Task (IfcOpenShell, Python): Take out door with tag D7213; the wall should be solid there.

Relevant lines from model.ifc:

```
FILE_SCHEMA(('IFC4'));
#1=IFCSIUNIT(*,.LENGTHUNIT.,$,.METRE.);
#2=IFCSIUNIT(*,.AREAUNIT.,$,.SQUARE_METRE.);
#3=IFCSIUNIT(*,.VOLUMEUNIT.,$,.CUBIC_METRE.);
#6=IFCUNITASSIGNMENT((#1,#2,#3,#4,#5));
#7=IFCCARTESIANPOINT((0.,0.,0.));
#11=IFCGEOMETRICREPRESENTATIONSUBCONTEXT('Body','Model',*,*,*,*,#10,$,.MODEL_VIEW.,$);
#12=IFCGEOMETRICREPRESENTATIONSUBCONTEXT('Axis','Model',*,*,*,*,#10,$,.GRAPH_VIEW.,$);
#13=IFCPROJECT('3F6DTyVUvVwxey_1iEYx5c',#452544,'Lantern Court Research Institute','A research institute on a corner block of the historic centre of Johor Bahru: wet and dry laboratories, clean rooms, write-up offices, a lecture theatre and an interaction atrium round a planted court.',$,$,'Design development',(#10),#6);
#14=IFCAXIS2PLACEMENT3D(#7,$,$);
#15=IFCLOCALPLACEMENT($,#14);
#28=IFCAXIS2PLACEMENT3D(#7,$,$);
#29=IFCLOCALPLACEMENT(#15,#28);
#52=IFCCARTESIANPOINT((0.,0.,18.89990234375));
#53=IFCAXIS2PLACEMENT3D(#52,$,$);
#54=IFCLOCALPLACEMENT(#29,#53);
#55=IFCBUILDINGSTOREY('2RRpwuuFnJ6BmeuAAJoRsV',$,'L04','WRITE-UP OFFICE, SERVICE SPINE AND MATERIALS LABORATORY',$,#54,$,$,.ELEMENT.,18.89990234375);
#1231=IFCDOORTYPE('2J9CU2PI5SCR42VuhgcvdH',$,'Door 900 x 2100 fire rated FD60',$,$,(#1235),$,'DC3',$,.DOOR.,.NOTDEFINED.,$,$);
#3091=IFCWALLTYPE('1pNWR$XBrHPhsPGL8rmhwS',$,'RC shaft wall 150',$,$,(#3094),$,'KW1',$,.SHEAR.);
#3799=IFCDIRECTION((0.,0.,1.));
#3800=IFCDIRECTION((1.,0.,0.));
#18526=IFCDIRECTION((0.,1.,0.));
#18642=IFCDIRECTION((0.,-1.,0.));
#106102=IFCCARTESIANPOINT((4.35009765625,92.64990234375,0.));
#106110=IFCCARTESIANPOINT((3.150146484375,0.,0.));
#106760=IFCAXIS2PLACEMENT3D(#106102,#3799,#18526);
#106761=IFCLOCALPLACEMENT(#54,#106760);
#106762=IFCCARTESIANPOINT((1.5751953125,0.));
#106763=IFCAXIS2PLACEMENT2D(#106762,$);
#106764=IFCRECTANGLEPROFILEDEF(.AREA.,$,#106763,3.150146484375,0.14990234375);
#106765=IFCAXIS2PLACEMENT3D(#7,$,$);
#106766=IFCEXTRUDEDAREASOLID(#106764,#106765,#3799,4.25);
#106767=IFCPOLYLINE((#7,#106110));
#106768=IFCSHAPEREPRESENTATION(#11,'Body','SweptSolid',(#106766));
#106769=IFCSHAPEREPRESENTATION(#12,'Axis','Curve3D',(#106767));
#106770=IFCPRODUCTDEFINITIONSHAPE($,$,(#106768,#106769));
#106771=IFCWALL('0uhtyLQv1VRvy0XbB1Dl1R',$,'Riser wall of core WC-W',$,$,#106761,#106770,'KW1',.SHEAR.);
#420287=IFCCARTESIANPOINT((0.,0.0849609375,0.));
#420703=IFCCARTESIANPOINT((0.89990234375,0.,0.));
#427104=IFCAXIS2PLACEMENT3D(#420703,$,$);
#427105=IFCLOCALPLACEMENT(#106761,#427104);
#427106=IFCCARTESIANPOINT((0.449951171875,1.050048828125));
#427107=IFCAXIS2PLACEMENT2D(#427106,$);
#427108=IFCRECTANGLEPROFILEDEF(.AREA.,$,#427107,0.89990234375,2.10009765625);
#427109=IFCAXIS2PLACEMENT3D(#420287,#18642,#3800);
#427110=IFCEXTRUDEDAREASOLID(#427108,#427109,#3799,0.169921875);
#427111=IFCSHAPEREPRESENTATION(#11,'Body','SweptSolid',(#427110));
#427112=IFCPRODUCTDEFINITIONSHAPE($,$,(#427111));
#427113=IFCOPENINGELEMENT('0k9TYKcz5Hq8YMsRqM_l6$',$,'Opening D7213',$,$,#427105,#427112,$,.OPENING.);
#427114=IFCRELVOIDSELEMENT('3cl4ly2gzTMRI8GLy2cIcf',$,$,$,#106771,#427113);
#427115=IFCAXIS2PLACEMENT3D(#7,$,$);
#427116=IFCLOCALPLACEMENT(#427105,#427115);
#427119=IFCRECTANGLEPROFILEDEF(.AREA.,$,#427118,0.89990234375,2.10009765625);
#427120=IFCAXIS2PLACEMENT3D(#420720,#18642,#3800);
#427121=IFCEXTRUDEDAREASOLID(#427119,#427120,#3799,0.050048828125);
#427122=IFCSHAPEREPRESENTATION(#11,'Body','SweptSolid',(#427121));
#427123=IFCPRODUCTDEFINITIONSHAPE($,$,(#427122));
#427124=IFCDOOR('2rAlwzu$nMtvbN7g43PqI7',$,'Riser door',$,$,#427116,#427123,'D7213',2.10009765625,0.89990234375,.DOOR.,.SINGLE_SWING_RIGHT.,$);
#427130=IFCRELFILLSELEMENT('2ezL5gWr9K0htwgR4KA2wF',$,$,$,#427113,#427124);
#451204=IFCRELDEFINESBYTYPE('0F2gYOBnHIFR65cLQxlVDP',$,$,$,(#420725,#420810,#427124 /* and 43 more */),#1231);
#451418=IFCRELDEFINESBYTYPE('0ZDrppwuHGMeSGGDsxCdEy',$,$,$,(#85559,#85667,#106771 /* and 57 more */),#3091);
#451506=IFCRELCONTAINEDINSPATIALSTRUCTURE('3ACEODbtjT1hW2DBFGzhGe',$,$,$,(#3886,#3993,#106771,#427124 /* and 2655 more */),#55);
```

```python
import ifcopenshell
import ifcopenshell.api.feature
import ifcopenshell.api.root
import ifcopenshell.geom
import ifcopenshell.util.shape

model = ifcopenshell.open("model.ifc")
settings = ifcopenshell.geom.settings()


def volume(element):
    """Net volume in cubic metres, openings subtracted."""
    shape = ifcopenshell.geom.create_shape(settings, element)
    return ifcopenshell.util.shape.get_volume(shape.geometry)


door = model.by_id(427124)
opening = door.FillsVoids[0].RelatingOpeningElement
wall = opening.VoidsElements[0].RelatingBuildingElement
before = volume(wall)

ifcopenshell.api.root.remove_product(model, product=door)
ifcopenshell.api.feature.remove_feature(model, feature=opening)

after = volume(wall)

print(f"wall volume {before:.3f} -> {after:.3f} m3")

model.write("model_v2.ifc")
```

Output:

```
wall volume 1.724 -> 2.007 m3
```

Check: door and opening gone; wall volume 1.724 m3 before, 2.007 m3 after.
